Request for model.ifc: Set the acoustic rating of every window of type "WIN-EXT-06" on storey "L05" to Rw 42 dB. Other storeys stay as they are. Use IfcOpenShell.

First a look at what the model holds.

```python
import ifcopenshell
import ifcopenshell.util.element

model = ifcopenshell.open("model.ifc")
print(model.schema)
storey = next(s for s in model.by_type("IfcBuildingStorey") if s.Name == "L05")
windows = [e for e in ifcopenshell.util.element.get_decomposition(storey) if e.is_a("IfcWindow")]
seen = {}
for e in windows:
    element_type = ifcopenshell.util.element.get_type(e)
    key = (element_type.Name if element_type != e and element_type else None, ifcopenshell.util.element.get_pset(e, "Pset_WindowCommon", "AcousticRating"))
    seen[key] = seen.get(key, 0) + 1
for (name, value), count in sorted(seen.items(), key=str):
    print(count, "x", name, "|", value)
```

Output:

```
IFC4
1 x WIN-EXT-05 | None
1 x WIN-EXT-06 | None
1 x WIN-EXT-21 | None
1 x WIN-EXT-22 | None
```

```python
import ifcopenshell
import ifcopenshell.api.pset
import ifcopenshell.util.element

model = ifcopenshell.open("model.ifc")

storey = next(s for s in model.by_type("IfcBuildingStorey") if s.Name == "L05")
windows = [e for e in ifcopenshell.util.element.get_decomposition(storey) if e.is_a("IfcWindow")]

count = 0
for e in windows:
    element_type = ifcopenshell.util.element.get_type(e)
    if element_type in (None, e) or element_type.Name != "WIN-EXT-06":
        continue
    # add_pset returns the element's existing set when there is one.
    pset = ifcopenshell.api.pset.add_pset(model, product=e, name="Pset_WindowCommon")
    ifcopenshell.api.pset.edit_pset(model, pset=pset, properties={"AcousticRating": "Rw 42 dB"})
    count += 1

print(count, "windows updated")

model.write("model_v2.ifc")
```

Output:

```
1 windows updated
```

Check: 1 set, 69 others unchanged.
